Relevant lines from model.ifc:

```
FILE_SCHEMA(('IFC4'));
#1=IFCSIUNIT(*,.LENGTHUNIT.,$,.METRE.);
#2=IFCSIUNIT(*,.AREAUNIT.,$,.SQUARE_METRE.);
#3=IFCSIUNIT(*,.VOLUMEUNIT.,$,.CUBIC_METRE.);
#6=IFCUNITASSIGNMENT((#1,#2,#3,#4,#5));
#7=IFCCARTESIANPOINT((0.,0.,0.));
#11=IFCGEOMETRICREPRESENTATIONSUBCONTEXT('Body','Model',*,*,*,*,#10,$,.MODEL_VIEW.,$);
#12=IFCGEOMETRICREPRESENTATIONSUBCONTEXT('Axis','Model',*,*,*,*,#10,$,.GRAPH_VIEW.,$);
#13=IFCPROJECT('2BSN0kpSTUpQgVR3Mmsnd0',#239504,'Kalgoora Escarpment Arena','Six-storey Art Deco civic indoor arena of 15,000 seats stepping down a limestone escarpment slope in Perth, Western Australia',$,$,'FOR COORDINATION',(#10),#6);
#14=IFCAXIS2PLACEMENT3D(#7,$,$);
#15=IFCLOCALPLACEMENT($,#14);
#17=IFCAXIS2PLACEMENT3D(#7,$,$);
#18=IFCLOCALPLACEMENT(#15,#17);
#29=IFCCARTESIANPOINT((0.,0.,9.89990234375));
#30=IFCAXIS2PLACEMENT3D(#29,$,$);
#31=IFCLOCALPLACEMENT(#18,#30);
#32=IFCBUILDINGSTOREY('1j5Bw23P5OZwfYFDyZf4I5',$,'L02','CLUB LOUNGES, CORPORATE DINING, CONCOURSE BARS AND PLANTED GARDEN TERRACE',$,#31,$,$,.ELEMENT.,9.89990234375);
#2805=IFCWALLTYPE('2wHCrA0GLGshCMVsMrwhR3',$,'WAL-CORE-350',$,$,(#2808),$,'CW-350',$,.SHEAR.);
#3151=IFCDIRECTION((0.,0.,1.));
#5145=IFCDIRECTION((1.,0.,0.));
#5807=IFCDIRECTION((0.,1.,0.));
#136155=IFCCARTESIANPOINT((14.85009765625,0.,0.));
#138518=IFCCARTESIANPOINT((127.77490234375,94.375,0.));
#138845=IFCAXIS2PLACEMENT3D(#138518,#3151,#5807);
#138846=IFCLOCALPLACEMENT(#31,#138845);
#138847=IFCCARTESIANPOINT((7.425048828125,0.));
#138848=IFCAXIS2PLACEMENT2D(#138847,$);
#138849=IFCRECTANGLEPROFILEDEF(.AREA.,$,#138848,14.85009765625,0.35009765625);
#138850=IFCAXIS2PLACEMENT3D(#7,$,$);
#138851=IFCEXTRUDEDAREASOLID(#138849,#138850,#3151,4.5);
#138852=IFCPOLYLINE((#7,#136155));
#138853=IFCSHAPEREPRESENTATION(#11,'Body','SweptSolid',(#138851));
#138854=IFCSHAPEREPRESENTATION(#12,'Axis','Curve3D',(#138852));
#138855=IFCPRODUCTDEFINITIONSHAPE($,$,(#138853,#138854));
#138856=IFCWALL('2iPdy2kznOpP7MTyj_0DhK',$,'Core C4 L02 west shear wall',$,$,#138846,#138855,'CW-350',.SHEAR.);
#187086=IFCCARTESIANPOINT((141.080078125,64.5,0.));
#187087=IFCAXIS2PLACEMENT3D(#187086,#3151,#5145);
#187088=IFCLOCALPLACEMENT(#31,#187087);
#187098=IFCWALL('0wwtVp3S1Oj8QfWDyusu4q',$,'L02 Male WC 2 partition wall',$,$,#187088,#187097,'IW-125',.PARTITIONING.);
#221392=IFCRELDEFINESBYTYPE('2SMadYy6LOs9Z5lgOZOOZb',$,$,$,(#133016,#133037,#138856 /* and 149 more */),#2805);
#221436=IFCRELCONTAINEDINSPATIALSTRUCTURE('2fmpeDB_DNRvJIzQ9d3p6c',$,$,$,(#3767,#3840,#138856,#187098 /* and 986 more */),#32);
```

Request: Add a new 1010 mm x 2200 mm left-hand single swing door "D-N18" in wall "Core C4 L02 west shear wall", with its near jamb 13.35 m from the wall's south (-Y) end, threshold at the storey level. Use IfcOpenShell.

```python
import numpy as np
import ifcopenshell
import ifcopenshell.api.feature
import ifcopenshell.api.geometry
import ifcopenshell.api.root
import ifcopenshell.api.spatial
import ifcopenshell.geom
import ifcopenshell.util.element
import ifcopenshell.util.placement
import ifcopenshell.util.representation
import ifcopenshell.util.shape
import ifcopenshell.util.unit

model = ifcopenshell.open("model.ifc")
unit_scale = ifcopenshell.util.unit.calculate_unit_scale(model)
settings = ifcopenshell.geom.settings()


def volume(element):
    """Net volume in cubic metres, openings subtracted."""
    shape = ifcopenshell.geom.create_shape(settings, element)
    return ifcopenshell.util.shape.get_volume(shape.geometry)


wall = model.by_guid("2iPdy2kznOpP7MTyj_0DhK")
storey = ifcopenshell.util.element.get_container(wall, ifc_class="IfcBuildingStorey")
context = ifcopenshell.util.representation.get_context(model, "Model", "Body", "MODEL_VIEW")
before = volume(wall)

width, height, from_end, sill = 1.01, 2.2, 13.35, 0.0  # metres

# The wall runs along its own X axis, and the end named is its -X end.
wall_shape = ifcopenshell.geom.create_shape(settings, wall)
x, y, z = ifcopenshell.util.shape.get_vertices(wall_shape.geometry).T
start = x.min() + from_end
face, thickness = float(y.min()), float(y.max() - y.min())
wall_matrix = ifcopenshell.util.placement.get_local_placement(wall.ObjectPlacement)
level = ifcopenshell.util.placement.get_local_placement(storey.ObjectPlacement)[2, 3]


def in_wall(x, y):
    """Placement at x, y metres in the wall's axes, at sill height."""
    matrix = wall_matrix.copy()
    matrix[:, 3] = wall_matrix @ np.array([x / unit_scale, y / unit_scale, 0.0, 1.0])
    matrix[2, 3] = level + sill / unit_scale
    return matrix


# Opening: a box that overshoots both wall faces by 50 mm.
opening = ifcopenshell.api.root.create_entity(model, ifc_class="IfcOpeningElement", predefined_type="OPENING")
box = ifcopenshell.api.geometry.add_wall_representation(
    model, context=context, length=width, height=height, thickness=thickness + 0.1
)
ifcopenshell.api.geometry.assign_representation(model, product=opening, representation=box)
ifcopenshell.api.geometry.edit_object_placement(model, product=opening, matrix=in_wall(start, face - 0.05), is_si=False)
ifcopenshell.api.feature.add_feature(model, feature=opening, element=wall)

door = ifcopenshell.api.root.create_entity(model, ifc_class="IfcDoor", name="D-N18", predefined_type="DOOR")
door.OverallWidth, door.OverallHeight = width / unit_scale, height / unit_scale
door.OperationType = "SINGLE_SWING_LEFT"
body = ifcopenshell.api.geometry.add_door_representation(
    model,
    context=context,
    overall_width=door.OverallWidth,
    overall_height=door.OverallHeight,
    operation_type="SINGLE_SWING_LEFT",
    lining_properties={"LiningDepth": thickness / unit_scale, "ThresholdDepth": thickness / unit_scale},
)
ifcopenshell.api.geometry.assign_representation(model, product=door, representation=body)
ifcopenshell.api.spatial.assign_container(model, products=[door], relating_structure=storey)
ifcopenshell.api.feature.add_filling(model, opening=opening, element=door)

# The lining spans the wall, so the door starts at the wall face.
ifcopenshell.api.geometry.edit_object_placement(model, product=door, matrix=in_wall(start, face), is_si=False)

after = volume(wall)

print(f"wall volume {before:.3f} -> {after:.3f} m3")

model.write("model_rev.ifc")
```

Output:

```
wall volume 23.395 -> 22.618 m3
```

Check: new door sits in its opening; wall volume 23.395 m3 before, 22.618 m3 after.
